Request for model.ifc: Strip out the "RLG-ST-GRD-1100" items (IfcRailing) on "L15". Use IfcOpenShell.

First a look at what the model holds.

```python
import ifcopenshell
import ifcopenshell.util.element

model = ifcopenshell.open("model.ifc")
print(model.schema)
storey = next(s for s in model.by_type("IfcBuildingStorey") if s.Name == "L15")
railings = [e for e in ifcopenshell.util.element.get_decomposition(storey) if e.is_a("IfcRailing")]
seen = {}
for e in railings:
    element_type = ifcopenshell.util.element.get_type(e)
    name = element_type.Name if element_type not in (None, e) else None
    seen[name] = seen.get(name, 0) + 1
for name, count in sorted(seen.items(), key=str):
    print(count, "x", name)
```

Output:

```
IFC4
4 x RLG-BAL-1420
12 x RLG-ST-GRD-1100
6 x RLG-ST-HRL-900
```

```python
import ifcopenshell
import ifcopenshell.api.root
import ifcopenshell.util.element

model = ifcopenshell.open("model.ifc")

storey = next(s for s in model.by_type("IfcBuildingStorey") if s.Name == "L15")
railings = [e for e in ifcopenshell.util.element.get_decomposition(storey) if e.is_a("IfcRailing")]
targets = [e for e in railings if (t := ifcopenshell.util.element.get_type(e)) not in (None, e) and t.Name == "RLG-ST-GRD-1100"]

for e in targets:
    ifcopenshell.api.root.remove_product(model, product=e)
print(len(targets), "removed")

model.write("model_v2.ifc")
```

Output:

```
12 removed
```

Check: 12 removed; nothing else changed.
